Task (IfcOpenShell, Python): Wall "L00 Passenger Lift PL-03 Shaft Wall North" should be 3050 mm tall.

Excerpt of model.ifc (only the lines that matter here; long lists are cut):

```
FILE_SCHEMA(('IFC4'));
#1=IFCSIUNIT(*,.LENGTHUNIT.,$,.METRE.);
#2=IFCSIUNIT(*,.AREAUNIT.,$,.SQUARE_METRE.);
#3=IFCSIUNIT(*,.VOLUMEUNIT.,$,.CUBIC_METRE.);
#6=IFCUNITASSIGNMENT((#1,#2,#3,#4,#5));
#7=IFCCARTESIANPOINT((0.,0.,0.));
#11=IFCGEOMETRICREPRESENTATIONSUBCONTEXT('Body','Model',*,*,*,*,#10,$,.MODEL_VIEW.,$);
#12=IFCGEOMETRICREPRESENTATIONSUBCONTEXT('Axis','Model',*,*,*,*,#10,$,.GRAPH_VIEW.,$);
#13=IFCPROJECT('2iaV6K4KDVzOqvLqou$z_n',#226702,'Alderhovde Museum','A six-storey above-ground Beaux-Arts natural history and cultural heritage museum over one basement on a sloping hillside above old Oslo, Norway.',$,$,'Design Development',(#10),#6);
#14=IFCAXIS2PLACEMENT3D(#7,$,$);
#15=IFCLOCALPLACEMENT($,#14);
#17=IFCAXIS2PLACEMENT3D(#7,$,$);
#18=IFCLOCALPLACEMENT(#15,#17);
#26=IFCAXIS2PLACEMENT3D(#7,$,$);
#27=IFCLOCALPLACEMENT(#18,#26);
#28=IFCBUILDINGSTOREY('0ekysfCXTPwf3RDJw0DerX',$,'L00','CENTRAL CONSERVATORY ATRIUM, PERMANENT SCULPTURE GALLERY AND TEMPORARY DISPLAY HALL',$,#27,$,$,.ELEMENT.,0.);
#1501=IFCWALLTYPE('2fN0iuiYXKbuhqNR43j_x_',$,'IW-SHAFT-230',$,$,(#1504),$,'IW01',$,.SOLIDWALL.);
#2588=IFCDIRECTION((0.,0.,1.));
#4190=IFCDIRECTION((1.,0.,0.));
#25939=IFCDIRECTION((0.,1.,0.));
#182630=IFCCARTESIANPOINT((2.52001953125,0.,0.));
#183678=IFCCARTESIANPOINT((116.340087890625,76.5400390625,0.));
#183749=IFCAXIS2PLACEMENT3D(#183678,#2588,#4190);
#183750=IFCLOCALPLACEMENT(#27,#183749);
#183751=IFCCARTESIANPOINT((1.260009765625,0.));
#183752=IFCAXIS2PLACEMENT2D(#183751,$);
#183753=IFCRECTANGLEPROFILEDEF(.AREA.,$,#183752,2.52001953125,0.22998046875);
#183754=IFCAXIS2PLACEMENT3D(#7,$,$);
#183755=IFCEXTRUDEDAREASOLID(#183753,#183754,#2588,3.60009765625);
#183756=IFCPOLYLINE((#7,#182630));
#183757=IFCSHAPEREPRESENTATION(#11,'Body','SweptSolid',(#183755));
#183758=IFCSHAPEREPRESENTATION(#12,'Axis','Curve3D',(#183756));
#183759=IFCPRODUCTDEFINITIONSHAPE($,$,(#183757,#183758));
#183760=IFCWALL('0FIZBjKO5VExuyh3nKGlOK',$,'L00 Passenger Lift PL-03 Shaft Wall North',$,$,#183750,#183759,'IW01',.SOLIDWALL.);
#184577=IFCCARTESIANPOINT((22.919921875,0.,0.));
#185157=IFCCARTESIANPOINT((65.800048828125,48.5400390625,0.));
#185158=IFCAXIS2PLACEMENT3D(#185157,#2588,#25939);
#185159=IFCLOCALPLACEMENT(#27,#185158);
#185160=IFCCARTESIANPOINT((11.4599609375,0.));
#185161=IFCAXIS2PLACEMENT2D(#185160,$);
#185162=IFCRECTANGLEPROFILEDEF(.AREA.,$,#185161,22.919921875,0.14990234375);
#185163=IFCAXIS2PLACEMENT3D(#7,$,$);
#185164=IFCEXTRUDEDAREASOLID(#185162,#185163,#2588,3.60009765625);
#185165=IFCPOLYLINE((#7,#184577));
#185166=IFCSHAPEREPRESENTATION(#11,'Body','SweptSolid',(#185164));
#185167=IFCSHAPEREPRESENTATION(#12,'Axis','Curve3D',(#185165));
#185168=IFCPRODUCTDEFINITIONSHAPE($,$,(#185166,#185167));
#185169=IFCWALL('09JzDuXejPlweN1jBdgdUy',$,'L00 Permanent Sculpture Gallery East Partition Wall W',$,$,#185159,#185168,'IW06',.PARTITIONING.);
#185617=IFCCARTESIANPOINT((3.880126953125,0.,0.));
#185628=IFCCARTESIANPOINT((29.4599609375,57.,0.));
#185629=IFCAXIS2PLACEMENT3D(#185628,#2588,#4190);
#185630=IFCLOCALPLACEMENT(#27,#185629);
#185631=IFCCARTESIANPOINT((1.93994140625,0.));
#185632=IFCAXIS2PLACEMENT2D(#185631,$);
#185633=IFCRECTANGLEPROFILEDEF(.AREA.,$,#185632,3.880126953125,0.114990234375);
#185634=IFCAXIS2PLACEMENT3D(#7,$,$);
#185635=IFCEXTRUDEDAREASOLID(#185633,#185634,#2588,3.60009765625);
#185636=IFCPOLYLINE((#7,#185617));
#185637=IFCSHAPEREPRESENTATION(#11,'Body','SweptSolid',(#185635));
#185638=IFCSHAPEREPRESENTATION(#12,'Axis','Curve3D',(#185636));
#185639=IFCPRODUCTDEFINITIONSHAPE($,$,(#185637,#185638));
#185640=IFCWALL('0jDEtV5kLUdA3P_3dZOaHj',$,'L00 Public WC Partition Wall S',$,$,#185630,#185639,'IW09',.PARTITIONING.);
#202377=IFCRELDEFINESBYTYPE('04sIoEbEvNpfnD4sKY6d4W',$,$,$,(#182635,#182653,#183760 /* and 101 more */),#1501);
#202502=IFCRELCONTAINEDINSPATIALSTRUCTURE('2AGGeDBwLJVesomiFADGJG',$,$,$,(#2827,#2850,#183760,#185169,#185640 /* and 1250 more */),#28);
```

```python
import ifcopenshell
import ifcopenshell.geom
import ifcopenshell.util.representation
import ifcopenshell.util.shape

model = ifcopenshell.open("model.ifc")
settings = ifcopenshell.geom.settings()


def volume(element):
    """Net volume in cubic metres, openings subtracted."""
    shape = ifcopenshell.geom.create_shape(settings, element)
    return ifcopenshell.util.shape.get_volume(shape.geometry)


wall = model.by_guid("0FIZBjKO5VExuyh3nKGlOK")
before = volume(wall)

body = ifcopenshell.util.representation.get_representation(wall, "Model", "Body")
solid = body.Items[0]
old_height = solid.Depth
solid.Depth = 3.05
after = volume(wall)

print(f"height {old_height:g} -> {solid.Depth:g}, volume {before:.3f} -> {after:.3f} m3")

model.write("model_rev.ifc")
```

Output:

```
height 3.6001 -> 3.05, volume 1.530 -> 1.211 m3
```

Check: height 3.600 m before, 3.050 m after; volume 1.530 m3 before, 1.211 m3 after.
